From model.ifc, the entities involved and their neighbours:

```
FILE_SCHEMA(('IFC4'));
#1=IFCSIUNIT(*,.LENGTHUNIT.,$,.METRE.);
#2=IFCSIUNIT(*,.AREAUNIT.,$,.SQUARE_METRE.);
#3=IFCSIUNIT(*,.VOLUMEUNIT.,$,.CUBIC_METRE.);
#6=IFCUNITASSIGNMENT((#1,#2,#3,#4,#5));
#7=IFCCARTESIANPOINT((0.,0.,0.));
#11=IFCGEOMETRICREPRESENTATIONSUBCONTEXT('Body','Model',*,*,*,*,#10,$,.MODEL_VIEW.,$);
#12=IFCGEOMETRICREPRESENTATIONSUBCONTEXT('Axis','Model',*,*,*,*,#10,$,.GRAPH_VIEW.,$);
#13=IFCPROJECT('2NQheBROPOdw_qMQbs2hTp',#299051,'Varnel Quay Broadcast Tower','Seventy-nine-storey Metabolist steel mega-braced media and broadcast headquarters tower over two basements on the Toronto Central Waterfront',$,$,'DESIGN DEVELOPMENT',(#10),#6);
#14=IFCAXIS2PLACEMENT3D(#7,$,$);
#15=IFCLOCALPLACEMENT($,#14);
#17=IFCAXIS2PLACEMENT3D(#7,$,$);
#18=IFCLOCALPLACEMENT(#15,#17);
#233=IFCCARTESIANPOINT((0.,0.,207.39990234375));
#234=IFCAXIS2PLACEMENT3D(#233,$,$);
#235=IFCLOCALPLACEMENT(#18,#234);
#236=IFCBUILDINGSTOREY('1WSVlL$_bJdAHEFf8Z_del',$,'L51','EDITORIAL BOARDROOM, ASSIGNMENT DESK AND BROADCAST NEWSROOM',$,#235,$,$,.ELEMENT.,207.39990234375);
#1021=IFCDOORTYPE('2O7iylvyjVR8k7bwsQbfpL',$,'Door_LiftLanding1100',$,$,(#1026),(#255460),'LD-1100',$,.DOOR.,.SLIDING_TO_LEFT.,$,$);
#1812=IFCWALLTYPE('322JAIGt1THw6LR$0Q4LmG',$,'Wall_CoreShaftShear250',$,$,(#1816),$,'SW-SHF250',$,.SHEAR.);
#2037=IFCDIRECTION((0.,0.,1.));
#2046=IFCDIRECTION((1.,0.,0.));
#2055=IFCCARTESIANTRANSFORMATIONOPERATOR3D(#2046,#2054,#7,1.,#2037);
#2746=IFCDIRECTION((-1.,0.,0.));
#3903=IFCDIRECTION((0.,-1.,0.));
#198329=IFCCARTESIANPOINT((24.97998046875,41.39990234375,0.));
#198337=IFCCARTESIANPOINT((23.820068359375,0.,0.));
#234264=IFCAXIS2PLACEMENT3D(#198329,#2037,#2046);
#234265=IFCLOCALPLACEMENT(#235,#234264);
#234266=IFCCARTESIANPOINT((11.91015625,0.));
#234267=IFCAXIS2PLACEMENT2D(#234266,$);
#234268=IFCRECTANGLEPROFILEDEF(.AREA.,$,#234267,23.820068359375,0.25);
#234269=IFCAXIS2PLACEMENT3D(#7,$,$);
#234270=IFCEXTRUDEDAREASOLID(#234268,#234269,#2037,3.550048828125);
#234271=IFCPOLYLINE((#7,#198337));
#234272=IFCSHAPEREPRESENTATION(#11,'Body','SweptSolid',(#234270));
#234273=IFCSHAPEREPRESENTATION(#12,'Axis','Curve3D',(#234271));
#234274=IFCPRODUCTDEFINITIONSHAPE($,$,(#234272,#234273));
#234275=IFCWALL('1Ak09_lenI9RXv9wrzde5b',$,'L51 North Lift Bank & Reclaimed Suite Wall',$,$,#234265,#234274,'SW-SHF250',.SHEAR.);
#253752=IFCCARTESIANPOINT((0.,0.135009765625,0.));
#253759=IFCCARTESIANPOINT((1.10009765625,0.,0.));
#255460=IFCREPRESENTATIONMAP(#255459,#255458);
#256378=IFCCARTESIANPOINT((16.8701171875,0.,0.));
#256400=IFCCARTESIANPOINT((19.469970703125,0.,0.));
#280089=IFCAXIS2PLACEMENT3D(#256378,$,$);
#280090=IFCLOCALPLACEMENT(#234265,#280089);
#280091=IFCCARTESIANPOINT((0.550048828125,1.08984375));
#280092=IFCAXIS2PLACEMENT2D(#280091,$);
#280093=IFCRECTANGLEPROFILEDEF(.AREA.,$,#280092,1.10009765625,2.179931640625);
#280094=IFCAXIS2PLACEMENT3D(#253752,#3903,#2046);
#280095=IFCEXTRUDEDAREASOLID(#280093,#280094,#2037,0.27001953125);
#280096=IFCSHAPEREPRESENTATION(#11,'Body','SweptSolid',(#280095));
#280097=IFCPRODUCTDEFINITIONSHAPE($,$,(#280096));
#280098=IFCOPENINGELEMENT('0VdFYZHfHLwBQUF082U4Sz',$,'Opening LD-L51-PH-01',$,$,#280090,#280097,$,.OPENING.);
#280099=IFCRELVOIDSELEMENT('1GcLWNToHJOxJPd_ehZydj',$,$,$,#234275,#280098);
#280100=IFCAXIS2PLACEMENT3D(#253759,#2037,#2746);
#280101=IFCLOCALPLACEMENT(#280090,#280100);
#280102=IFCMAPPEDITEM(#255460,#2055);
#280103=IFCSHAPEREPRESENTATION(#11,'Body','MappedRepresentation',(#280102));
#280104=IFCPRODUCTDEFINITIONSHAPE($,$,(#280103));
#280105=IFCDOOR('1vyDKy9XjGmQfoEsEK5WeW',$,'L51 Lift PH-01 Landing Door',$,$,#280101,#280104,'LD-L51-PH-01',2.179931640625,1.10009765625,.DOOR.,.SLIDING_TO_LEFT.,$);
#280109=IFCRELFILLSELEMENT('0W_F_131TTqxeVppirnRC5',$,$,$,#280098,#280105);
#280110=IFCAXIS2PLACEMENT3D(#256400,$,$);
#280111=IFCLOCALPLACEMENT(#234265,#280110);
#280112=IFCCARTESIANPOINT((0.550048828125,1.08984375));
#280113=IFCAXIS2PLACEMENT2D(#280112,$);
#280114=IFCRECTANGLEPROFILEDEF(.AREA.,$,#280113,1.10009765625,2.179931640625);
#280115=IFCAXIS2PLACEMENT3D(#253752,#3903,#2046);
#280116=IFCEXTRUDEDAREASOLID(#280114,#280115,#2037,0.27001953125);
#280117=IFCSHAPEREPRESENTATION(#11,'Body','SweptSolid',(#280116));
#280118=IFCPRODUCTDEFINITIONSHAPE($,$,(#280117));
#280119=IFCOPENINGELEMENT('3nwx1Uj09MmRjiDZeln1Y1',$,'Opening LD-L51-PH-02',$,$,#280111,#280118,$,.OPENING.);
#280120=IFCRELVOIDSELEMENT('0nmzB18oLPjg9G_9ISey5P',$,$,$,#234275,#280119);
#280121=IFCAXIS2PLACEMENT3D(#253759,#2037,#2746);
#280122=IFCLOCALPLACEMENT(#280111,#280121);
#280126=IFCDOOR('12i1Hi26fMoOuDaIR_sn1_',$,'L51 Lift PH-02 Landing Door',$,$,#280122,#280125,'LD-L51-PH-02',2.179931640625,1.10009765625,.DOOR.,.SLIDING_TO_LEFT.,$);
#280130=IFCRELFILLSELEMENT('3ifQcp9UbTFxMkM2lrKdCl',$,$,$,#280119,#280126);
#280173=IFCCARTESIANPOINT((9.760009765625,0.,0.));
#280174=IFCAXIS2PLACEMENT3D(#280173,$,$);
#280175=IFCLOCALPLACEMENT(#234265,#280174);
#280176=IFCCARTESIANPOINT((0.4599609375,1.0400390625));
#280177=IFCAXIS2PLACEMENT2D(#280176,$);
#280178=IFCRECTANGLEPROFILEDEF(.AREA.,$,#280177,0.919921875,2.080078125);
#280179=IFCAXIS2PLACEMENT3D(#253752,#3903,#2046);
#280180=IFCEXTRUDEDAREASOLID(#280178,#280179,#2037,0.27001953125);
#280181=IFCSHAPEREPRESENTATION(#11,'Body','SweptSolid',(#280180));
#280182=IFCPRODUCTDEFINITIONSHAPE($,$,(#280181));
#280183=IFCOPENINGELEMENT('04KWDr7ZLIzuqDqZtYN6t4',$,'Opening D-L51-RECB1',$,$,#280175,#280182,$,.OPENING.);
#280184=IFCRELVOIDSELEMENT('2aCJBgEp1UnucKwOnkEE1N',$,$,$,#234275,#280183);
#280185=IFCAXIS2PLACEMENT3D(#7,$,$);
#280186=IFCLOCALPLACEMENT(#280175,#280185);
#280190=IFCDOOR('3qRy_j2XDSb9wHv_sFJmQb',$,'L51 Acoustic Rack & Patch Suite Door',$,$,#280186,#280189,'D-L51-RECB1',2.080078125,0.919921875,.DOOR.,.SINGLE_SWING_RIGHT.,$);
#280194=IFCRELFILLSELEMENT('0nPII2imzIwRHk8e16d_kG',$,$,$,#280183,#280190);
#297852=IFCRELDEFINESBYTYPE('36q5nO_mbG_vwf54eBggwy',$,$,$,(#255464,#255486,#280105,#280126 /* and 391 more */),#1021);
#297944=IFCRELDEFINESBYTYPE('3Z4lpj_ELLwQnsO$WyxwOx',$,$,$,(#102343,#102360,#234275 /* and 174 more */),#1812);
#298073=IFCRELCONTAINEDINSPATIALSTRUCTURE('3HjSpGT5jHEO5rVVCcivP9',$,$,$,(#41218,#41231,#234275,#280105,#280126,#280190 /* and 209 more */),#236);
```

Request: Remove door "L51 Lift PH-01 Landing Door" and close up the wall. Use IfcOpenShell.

```python
import ifcopenshell
import ifcopenshell.api.feature
import ifcopenshell.api.root
import ifcopenshell.geom
import ifcopenshell.util.shape

model = ifcopenshell.open("model.ifc")
settings = ifcopenshell.geom.settings()


def volume(element):
    """Net volume in cubic metres, openings subtracted."""
    shape = ifcopenshell.geom.create_shape(settings, element)
    return ifcopenshell.util.shape.get_volume(shape.geometry)


door = model.by_guid("1vyDKy9XjGmQfoEsEK5WeW")
opening = door.FillsVoids[0].RelatingOpeningElement
wall = opening.VoidsElements[0].RelatingBuildingElement
before = volume(wall)

ifcopenshell.api.root.remove_product(model, product=door)
ifcopenshell.api.feature.remove_feature(model, feature=opening)

after = volume(wall)

print(f"wall volume {before:.3f} -> {after:.3f} m3")

model.write("model_edited.ifc")
```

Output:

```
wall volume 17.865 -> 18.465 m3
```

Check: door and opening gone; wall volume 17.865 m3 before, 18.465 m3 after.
